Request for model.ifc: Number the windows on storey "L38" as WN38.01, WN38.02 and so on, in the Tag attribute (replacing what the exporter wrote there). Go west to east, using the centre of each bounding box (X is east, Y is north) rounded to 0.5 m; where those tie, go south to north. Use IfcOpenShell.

First a look at what the model holds.

```python
import ifcopenshell
import ifcopenshell.util.element
import ifcopenshell.util.placement

model = ifcopenshell.open("model.ifc")
print(model.schema)
storey = next(s for s in model.by_type("IfcBuildingStorey") if s.Name == "L38")
windows = [e for e in ifcopenshell.util.element.get_decomposition(storey) if e.is_a("IfcWindow")]
for e in sorted(windows, key=lambda e: e.id()):
    origin = ifcopenshell.util.placement.get_local_placement(e.ObjectPlacement)[:3, 3]
    print(e.id(), e.Tag, e.Name, origin.round(2) + 0.0, sep=" | ")
```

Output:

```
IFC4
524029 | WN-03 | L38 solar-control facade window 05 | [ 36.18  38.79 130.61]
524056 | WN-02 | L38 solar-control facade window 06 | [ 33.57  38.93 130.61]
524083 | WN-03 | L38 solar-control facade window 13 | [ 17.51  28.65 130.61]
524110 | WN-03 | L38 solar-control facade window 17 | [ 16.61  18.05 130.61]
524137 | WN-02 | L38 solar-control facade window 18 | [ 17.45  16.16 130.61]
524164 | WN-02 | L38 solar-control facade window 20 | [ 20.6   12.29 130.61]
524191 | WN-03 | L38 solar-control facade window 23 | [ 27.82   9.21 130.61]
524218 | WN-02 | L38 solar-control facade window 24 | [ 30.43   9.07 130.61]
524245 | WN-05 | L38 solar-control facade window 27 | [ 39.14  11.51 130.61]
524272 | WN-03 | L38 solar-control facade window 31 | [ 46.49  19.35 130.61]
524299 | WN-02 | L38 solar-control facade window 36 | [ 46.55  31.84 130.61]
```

```python
import ifcopenshell
import ifcopenshell.geom
import ifcopenshell.util.element
import ifcopenshell.util.shape

model = ifcopenshell.open("model.ifc")
settings = ifcopenshell.geom.settings()
settings.set("use-world-coords", True)


def centre(element):
    shape = ifcopenshell.geom.create_shape(settings, element)
    return ifcopenshell.util.shape.get_bbox_centroid(shape.geometry)


storey = next(s for s in model.by_type("IfcBuildingStorey") if s.Name == "L38")
windows = [e for e in ifcopenshell.util.element.get_decomposition(storey) if e.is_a("IfcWindow")]

# Insertion points can sit at a corner or the storey origin, so sort by the geometry (in metres).
centres = {e: centre(e) for e in windows}
windows.sort(key=lambda e: (round(centres[e][0] / 0.5), centres[e][1]))

for i, e in enumerate(windows, start=1):
    number = f"WN38.{i:02d}"
    e.Tag = number
    print(e.id(), number)

model.write("model_v2.ifc")
```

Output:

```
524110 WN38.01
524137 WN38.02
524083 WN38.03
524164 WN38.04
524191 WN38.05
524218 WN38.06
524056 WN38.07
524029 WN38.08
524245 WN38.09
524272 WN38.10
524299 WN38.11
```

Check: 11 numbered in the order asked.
